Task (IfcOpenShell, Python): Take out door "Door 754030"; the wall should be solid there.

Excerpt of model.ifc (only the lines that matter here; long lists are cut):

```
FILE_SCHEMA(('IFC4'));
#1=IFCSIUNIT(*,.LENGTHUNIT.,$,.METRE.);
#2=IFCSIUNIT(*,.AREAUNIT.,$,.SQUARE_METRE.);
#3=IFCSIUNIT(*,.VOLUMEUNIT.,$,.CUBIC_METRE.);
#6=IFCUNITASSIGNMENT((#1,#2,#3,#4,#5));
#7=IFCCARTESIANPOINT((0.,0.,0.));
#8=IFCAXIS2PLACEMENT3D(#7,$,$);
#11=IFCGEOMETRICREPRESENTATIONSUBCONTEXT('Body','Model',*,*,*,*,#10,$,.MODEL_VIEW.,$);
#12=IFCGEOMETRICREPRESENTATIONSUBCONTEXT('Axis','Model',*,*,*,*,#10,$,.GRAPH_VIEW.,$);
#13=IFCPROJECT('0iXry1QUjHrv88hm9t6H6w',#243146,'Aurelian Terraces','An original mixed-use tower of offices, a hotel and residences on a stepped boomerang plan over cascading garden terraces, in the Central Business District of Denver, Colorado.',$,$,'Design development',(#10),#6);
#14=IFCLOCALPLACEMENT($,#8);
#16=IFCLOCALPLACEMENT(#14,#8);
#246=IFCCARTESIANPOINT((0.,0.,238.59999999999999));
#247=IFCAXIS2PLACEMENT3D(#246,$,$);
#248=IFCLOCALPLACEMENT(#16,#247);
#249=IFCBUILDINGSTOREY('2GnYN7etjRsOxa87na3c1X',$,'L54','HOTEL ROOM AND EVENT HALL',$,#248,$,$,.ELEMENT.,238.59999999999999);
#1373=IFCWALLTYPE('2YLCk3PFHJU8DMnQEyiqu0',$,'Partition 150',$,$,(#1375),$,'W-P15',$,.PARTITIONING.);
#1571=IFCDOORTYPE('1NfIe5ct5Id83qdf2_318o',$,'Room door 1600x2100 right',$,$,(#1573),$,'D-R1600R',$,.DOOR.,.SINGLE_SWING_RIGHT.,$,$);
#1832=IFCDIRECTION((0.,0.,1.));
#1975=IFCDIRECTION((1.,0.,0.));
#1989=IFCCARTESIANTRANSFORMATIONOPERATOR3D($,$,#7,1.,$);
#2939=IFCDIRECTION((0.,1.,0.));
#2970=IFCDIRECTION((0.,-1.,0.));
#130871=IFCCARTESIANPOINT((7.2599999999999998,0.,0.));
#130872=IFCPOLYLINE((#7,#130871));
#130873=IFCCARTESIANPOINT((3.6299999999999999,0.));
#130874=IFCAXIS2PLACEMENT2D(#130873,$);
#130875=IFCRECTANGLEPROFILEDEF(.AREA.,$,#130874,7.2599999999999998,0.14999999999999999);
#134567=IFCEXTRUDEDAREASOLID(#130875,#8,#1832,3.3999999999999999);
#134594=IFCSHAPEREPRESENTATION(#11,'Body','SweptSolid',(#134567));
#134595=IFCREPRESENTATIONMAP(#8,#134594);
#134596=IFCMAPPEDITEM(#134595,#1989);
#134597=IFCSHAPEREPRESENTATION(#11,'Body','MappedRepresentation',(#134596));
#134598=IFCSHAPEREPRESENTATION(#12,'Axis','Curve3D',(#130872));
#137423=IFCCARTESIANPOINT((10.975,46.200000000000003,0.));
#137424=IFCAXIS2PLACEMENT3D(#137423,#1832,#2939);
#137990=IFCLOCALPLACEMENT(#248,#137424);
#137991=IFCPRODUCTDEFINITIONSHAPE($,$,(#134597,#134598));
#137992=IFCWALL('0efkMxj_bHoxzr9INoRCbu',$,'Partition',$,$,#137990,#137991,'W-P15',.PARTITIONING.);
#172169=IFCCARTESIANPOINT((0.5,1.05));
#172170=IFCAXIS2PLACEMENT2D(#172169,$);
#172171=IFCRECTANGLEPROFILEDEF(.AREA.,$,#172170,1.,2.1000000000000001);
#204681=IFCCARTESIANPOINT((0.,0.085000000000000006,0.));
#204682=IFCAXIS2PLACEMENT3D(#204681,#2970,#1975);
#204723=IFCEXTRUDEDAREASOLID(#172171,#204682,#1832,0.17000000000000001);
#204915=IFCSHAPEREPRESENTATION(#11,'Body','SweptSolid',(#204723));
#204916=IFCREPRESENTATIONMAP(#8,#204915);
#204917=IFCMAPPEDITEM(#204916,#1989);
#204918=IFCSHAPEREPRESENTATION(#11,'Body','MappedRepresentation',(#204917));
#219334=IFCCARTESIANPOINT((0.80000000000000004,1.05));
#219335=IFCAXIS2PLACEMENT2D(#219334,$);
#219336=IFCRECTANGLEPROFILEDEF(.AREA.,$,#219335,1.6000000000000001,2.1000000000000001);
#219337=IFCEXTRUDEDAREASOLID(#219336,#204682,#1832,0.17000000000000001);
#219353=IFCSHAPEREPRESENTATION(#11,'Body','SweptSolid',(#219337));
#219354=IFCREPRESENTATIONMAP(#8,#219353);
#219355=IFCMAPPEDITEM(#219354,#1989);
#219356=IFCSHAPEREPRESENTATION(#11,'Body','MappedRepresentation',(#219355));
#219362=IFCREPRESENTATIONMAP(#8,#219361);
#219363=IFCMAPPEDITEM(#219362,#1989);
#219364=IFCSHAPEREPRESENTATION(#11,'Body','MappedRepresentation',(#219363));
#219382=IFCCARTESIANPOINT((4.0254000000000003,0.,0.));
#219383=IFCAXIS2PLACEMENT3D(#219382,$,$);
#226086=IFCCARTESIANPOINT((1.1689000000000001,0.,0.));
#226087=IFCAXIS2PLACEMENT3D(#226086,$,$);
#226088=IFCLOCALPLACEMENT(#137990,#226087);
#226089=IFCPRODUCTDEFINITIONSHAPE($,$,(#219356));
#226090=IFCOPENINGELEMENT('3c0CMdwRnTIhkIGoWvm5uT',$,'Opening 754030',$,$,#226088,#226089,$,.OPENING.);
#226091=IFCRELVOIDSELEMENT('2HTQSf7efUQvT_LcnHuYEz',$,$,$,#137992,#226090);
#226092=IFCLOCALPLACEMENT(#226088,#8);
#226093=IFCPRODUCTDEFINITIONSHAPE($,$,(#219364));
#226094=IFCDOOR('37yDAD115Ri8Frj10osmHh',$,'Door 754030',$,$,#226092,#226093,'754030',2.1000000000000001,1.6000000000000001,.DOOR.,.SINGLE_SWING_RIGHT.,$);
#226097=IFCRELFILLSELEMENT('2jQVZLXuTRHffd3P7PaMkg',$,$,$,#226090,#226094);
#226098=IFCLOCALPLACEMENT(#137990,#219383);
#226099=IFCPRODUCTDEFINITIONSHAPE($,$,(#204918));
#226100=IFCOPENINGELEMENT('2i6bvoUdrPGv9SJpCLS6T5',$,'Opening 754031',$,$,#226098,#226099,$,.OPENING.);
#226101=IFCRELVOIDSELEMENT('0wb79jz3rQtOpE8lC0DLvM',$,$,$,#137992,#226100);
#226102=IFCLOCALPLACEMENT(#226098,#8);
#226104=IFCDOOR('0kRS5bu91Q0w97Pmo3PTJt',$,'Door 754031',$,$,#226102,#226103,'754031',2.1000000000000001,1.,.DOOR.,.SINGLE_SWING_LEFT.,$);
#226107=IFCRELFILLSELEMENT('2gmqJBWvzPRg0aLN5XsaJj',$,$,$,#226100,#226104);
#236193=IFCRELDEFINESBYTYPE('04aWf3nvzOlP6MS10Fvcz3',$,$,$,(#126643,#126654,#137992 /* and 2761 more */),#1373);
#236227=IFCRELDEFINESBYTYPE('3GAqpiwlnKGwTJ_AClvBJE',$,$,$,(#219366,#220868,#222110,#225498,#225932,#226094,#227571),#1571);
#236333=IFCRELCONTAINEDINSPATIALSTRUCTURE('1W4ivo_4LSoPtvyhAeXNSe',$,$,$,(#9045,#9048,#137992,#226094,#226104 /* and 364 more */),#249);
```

```python
import ifcopenshell
import ifcopenshell.api.feature
import ifcopenshell.api.root
import ifcopenshell.geom
import ifcopenshell.util.shape

model = ifcopenshell.open("model.ifc")
settings = ifcopenshell.geom.settings()


def volume(element):
    """Net volume in cubic metres, openings subtracted."""
    shape = ifcopenshell.geom.create_shape(settings, element)
    return ifcopenshell.util.shape.get_volume(shape.geometry)


door = model.by_id(226094)
opening = door.FillsVoids[0].RelatingOpeningElement
wall = opening.VoidsElements[0].RelatingBuildingElement
before = volume(wall)

ifcopenshell.api.root.remove_product(model, product=door)
ifcopenshell.api.feature.remove_feature(model, feature=opening)

after = volume(wall)

print(f"wall volume {before:.3f} -> {after:.3f} m3")

model.write("model_rev.ifc")
```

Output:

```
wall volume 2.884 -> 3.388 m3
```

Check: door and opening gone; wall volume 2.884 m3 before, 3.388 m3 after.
